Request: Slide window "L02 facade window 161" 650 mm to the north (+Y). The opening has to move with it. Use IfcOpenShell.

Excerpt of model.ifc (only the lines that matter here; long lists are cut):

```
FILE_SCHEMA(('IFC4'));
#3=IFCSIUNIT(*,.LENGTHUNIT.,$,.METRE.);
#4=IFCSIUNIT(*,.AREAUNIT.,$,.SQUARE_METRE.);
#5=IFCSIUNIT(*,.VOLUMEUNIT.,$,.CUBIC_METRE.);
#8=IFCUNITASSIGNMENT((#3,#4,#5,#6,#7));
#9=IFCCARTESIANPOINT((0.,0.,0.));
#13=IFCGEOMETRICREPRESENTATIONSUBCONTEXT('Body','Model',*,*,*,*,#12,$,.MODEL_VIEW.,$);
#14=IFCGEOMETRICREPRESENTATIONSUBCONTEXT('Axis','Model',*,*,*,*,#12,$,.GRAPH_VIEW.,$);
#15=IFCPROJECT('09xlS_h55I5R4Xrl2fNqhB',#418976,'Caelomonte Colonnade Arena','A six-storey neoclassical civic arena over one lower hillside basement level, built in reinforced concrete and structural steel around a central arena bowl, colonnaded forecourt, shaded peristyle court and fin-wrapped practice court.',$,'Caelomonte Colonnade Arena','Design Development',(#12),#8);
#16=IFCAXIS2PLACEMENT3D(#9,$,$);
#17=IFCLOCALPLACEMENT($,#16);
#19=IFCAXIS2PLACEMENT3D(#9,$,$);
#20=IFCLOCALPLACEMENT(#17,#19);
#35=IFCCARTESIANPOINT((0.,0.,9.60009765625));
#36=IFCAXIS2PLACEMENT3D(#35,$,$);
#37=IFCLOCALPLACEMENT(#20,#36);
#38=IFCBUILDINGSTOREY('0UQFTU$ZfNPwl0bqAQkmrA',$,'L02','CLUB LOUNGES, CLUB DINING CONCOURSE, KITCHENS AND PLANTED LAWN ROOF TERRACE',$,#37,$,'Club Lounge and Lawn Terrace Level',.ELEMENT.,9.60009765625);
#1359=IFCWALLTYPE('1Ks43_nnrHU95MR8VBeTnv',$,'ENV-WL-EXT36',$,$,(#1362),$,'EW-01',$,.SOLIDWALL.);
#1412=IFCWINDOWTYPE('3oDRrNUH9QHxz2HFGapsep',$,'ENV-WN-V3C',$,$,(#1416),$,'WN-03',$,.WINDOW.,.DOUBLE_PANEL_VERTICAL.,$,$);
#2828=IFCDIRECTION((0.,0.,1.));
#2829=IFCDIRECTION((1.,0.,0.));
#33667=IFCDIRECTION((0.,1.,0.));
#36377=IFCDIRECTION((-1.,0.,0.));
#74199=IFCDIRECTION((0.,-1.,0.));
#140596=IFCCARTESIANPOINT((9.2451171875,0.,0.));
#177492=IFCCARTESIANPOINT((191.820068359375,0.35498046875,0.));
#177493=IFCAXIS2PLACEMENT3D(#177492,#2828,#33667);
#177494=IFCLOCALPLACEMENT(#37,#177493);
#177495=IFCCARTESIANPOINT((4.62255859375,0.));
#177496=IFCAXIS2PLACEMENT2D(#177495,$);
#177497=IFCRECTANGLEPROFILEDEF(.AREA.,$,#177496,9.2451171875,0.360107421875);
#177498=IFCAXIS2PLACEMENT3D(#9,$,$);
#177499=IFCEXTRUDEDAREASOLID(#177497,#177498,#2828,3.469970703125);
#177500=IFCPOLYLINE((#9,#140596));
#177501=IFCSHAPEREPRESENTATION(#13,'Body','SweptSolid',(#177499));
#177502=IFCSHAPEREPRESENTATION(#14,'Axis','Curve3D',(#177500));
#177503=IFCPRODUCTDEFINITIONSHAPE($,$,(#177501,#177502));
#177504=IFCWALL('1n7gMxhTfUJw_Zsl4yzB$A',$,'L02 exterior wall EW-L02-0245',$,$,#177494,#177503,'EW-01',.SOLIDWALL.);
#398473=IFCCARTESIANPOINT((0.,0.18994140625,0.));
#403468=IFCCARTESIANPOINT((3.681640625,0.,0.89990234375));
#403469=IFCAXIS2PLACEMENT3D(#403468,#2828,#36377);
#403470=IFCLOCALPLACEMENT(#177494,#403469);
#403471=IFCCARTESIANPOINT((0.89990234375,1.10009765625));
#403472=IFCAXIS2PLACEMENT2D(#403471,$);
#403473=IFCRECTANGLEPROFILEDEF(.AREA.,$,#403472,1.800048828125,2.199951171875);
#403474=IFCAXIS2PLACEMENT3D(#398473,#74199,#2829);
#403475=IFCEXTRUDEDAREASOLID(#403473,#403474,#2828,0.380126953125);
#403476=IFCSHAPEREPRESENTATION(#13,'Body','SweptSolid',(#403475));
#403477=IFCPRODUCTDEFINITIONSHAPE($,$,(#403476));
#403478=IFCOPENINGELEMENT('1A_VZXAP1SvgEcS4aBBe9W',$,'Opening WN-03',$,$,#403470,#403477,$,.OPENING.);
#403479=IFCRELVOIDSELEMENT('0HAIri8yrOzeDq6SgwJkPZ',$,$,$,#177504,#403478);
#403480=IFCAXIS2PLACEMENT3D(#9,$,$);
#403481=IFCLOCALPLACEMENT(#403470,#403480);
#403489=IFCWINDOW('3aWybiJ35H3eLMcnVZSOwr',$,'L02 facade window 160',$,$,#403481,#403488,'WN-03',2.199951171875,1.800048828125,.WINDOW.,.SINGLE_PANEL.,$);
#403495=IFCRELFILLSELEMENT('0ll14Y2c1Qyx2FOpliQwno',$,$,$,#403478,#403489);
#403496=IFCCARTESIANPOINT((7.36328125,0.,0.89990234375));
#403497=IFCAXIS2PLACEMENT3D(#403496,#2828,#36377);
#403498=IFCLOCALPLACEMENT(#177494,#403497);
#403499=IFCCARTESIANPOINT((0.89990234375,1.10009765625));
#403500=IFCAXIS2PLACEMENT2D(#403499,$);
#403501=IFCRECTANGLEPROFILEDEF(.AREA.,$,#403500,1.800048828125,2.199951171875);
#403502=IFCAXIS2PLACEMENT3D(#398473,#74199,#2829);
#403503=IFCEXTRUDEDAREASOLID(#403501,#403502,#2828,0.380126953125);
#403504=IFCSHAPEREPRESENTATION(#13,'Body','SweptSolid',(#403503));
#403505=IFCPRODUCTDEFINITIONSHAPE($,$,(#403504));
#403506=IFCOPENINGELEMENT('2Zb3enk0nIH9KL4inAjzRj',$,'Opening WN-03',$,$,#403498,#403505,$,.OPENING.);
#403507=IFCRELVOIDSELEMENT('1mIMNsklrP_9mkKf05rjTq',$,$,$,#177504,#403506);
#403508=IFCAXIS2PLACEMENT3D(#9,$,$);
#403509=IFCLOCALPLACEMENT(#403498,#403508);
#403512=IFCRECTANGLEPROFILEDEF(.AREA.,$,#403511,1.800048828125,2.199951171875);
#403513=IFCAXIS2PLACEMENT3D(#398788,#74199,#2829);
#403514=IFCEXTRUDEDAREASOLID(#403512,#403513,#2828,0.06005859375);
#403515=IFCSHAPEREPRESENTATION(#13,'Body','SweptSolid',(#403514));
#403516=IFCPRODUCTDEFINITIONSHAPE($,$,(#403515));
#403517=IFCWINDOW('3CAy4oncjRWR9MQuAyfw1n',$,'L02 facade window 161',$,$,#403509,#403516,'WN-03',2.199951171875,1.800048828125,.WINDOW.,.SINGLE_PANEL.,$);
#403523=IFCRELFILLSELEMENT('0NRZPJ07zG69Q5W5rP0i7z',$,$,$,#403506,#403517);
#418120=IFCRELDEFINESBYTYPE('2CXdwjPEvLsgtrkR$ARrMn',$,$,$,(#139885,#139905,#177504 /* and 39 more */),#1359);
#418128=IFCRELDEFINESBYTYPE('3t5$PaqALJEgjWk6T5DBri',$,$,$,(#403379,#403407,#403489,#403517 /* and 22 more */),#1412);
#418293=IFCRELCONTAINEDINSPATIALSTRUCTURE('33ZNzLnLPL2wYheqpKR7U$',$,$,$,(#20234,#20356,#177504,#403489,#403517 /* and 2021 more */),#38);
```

```python
import ifcopenshell
import ifcopenshell.api.geometry
import ifcopenshell.util.placement
import ifcopenshell.util.unit

model = ifcopenshell.open("model.ifc")
unit_scale = ifcopenshell.util.unit.calculate_unit_scale(model)

window = model.by_id(403517)
opening = window.FillsVoids[0].RelatingOpeningElement
wall = opening.VoidsElements[0].RelatingBuildingElement

wall_matrix = ifcopenshell.util.placement.get_local_placement(wall.ObjectPlacement)
shift = wall_matrix[:3, 0] * 0.65 / unit_scale
before = ifcopenshell.util.placement.get_local_placement(window.ObjectPlacement)[:3, 3].copy()

# The window is placed relative to its opening, so it follows when the opening moves.
matrix = ifcopenshell.util.placement.get_local_placement(opening.ObjectPlacement)
matrix[:3, 3] += shift
ifcopenshell.api.geometry.edit_object_placement(
    model, product=opening, matrix=matrix, is_si=False, should_transform_children=True
)

after = ifcopenshell.util.placement.get_local_placement(window.ObjectPlacement)[:3, 3]
print("window moved by", (after - before).round(3) + 0.0)

model.write("model_rev.ifc")
```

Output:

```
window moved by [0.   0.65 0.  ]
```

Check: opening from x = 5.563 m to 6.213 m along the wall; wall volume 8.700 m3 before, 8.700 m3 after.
